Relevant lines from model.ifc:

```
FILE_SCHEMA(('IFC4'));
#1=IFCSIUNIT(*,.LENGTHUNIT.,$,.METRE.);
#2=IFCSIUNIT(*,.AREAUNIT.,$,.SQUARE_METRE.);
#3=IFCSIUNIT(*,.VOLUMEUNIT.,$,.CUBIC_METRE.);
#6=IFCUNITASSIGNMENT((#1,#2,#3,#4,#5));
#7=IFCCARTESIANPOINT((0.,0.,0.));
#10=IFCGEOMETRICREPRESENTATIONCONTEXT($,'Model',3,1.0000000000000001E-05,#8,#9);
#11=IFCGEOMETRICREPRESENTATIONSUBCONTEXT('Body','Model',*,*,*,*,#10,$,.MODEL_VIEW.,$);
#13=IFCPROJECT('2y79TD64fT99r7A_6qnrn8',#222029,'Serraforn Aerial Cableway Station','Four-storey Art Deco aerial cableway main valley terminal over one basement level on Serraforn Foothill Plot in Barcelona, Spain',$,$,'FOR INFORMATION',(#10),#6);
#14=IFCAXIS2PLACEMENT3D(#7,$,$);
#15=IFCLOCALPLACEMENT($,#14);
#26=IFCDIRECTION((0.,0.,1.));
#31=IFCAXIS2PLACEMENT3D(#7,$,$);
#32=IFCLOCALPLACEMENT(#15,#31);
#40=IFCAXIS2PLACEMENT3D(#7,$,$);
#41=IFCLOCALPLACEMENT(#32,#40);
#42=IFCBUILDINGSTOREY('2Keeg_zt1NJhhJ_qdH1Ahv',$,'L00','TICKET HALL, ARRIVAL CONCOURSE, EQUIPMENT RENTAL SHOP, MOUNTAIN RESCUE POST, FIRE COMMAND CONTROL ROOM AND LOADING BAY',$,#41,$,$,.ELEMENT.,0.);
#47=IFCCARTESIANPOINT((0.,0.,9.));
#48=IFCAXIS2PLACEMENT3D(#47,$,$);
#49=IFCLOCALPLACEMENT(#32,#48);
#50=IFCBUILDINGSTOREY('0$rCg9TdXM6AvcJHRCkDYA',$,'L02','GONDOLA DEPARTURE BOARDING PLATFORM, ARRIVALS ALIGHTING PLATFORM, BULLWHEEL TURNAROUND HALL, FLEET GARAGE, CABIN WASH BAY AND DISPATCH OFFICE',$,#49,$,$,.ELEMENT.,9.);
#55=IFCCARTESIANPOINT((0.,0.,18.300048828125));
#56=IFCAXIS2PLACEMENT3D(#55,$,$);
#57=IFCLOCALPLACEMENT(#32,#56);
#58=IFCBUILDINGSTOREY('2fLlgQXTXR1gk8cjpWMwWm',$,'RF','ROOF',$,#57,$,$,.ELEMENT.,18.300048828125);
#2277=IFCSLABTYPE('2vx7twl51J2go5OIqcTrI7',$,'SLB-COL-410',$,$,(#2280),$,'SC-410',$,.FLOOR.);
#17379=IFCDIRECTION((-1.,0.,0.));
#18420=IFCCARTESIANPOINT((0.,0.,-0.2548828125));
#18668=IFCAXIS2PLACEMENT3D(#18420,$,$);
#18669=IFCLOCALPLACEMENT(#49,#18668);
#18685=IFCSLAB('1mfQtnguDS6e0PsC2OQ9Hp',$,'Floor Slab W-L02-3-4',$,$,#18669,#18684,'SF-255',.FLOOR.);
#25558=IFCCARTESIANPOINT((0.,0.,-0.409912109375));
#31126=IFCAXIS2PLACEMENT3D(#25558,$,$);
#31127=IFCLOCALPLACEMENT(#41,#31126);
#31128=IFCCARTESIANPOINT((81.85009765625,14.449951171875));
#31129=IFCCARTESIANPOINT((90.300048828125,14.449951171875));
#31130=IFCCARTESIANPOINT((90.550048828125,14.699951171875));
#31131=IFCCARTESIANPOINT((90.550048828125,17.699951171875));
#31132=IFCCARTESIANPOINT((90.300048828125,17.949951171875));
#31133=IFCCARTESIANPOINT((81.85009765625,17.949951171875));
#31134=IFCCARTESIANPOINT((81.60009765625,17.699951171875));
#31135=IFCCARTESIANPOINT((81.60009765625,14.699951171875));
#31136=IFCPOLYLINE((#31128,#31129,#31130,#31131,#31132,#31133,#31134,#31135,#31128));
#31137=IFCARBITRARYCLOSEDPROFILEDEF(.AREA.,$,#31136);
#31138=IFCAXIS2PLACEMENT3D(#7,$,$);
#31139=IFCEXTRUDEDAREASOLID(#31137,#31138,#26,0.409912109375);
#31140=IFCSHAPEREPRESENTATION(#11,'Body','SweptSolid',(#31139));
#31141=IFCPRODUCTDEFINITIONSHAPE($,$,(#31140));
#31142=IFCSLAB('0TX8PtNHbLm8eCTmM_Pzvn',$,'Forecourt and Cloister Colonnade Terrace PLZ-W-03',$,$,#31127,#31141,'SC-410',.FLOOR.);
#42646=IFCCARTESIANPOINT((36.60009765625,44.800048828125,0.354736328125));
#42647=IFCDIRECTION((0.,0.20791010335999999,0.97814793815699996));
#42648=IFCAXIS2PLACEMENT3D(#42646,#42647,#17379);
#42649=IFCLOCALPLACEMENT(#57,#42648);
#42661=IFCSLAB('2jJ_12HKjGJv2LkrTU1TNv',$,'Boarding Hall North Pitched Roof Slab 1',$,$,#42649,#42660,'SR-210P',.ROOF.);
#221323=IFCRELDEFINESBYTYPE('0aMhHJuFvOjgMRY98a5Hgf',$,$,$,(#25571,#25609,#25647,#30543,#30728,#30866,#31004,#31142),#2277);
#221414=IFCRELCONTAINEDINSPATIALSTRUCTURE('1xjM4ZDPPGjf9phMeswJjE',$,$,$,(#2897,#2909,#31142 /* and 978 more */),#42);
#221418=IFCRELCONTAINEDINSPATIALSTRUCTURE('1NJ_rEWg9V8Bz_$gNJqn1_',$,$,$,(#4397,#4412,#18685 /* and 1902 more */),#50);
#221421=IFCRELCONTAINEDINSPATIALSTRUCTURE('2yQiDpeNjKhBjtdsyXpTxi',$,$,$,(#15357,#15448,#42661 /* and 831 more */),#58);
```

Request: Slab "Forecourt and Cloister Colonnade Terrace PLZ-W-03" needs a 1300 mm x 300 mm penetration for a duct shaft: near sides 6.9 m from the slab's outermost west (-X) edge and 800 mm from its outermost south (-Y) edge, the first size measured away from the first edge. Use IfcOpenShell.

```python
import numpy as np
import ifcopenshell
import ifcopenshell.api.feature
import ifcopenshell.api.geometry
import ifcopenshell.api.root
import ifcopenshell.geom
import ifcopenshell.util.placement
import ifcopenshell.util.representation
import ifcopenshell.util.shape
import ifcopenshell.util.unit

model = ifcopenshell.open("model.ifc")
unit_scale = ifcopenshell.util.unit.calculate_unit_scale(model)
settings = ifcopenshell.geom.settings()


def volume(element):
    """Net volume in cubic metres, openings subtracted."""
    shape = ifcopenshell.geom.create_shape(settings, element)
    return ifcopenshell.util.shape.get_volume(shape.geometry)


slab = model.by_guid("0TX8PtNHbLm8eCTmM_Pzvn")
before = volume(slab)

# Extent in the slab's own axes, in metres. The edges named are its -X and -Y sides.
slab_shape = ifcopenshell.geom.create_shape(settings, slab)
vertices = ifcopenshell.util.shape.get_vertices(slab_shape.geometry)
x_min, y_min, bottom = vertices.min(axis=0)
top = vertices[:, 2].max()

opening = ifcopenshell.api.root.create_entity(model, ifc_class="IfcOpeningElement", name="Duct shaft opening", predefined_type="OPENING")
context = ifcopenshell.util.representation.get_context(model, "Model", "Body", "MODEL_VIEW")
width, depth = 1.3, 0.3
outline = [(0.0, 0.0), (width, 0.0), (width, depth), (0.0, depth), (0.0, 0.0)]
# Overshoot both faces by 50 mm so the cut is clean.
shape = ifcopenshell.api.geometry.add_slab_representation(
    model, context=context, depth=top - bottom + 0.1, polyline=outline
)
ifcopenshell.api.geometry.assign_representation(model, product=opening, representation=shape)

matrix = ifcopenshell.util.placement.get_local_placement(slab.ObjectPlacement)
matrix[:, 3] = matrix @ np.append(np.array([x_min + 6.9, y_min + 0.8, bottom - 0.05]) / unit_scale, 1.0)
ifcopenshell.api.geometry.edit_object_placement(model, product=opening, matrix=matrix, is_si=False)
ifcopenshell.api.feature.add_feature(model, feature=opening, element=slab)

after = volume(slab)

print(f"slab volume {before:.3f} -> {after:.3f} m3")

model.write("model_v2.ifc")
```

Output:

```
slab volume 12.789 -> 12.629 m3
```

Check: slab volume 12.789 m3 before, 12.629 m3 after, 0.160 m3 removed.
